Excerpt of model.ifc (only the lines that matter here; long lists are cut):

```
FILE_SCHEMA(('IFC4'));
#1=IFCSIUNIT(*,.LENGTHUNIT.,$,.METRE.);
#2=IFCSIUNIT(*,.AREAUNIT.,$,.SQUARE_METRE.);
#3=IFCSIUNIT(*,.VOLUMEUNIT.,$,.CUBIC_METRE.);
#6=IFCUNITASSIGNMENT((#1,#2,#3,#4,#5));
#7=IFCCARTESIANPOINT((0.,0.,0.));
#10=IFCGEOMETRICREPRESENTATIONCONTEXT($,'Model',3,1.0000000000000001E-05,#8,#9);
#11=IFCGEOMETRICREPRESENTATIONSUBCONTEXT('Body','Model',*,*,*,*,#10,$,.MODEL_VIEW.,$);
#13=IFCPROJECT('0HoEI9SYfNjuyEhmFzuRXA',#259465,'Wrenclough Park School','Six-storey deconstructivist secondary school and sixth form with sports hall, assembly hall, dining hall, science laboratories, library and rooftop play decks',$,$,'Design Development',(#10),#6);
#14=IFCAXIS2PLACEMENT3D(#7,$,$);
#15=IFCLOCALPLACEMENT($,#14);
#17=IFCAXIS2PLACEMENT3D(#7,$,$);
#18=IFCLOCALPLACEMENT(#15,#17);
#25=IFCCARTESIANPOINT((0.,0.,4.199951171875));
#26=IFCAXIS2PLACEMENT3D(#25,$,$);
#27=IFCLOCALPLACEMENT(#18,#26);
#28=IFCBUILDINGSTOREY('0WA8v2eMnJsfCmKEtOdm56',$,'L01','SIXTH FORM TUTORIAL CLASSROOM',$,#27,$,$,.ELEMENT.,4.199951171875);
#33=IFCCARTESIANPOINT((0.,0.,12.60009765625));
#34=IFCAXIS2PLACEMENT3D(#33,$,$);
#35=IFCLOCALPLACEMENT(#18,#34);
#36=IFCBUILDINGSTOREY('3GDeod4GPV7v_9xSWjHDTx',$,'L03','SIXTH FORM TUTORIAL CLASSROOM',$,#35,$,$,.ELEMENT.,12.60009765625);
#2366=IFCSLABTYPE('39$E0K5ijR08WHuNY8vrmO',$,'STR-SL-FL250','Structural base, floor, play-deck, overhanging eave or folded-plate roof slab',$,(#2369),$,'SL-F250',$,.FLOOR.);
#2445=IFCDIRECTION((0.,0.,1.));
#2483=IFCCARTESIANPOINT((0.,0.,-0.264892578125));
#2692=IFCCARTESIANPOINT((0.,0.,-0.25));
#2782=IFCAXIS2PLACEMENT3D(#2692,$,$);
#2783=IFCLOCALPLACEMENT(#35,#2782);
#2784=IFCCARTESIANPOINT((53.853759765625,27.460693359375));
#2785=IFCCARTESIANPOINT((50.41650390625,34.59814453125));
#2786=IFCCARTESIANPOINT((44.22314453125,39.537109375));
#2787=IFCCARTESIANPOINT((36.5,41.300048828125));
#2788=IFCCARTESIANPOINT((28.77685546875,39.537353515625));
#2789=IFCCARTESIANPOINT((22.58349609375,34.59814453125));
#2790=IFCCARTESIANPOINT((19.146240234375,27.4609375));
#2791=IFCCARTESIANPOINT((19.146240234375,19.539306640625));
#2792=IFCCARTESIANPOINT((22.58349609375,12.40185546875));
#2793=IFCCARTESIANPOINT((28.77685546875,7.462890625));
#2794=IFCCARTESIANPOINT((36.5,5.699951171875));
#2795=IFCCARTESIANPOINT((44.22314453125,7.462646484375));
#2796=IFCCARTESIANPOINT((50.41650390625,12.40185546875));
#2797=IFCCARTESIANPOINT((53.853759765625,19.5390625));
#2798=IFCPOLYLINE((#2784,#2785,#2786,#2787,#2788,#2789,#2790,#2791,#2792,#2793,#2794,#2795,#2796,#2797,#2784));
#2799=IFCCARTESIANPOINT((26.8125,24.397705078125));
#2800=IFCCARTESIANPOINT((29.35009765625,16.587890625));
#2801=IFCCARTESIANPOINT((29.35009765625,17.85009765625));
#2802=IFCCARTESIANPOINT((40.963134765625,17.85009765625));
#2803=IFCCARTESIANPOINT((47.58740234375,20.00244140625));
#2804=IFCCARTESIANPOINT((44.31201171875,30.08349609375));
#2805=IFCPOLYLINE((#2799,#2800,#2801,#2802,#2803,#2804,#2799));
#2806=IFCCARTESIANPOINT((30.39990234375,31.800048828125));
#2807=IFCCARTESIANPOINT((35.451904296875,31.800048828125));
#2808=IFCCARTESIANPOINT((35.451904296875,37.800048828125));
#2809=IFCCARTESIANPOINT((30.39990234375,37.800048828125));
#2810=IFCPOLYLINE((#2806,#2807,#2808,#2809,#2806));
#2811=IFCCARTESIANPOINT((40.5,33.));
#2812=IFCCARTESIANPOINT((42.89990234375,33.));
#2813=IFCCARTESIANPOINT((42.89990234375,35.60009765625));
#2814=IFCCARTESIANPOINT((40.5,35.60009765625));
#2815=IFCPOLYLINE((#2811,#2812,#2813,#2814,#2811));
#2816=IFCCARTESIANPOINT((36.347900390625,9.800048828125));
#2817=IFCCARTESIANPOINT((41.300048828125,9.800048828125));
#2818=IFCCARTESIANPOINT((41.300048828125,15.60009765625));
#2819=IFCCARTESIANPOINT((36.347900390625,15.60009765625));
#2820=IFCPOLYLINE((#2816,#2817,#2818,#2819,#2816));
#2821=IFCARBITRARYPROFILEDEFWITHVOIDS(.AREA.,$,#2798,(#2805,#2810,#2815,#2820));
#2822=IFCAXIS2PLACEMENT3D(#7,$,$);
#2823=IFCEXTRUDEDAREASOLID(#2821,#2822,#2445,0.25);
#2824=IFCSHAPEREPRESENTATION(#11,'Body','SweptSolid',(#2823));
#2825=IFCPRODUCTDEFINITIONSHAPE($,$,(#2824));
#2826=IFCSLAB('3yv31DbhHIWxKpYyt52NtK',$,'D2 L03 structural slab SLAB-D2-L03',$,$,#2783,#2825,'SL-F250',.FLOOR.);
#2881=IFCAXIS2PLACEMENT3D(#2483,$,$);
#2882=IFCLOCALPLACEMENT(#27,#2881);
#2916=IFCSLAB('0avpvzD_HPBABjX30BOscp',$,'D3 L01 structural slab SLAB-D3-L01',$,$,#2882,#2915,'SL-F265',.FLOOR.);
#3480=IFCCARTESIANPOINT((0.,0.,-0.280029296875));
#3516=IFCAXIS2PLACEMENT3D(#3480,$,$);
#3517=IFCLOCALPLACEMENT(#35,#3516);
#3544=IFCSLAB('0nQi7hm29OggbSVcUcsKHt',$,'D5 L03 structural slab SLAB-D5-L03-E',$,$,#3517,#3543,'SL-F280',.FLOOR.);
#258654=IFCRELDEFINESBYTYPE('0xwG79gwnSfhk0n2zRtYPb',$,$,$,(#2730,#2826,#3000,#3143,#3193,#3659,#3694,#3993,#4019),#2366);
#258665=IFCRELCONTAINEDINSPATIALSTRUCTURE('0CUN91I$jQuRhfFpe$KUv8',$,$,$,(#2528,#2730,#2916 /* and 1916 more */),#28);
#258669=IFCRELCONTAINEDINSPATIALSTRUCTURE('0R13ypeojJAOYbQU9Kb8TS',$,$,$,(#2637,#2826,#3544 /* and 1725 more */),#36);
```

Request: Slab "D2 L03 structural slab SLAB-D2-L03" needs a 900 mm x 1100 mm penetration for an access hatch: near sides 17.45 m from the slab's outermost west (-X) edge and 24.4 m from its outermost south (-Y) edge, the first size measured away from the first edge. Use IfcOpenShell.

```python
import numpy as np
import ifcopenshell
import ifcopenshell.api.feature
import ifcopenshell.api.geometry
import ifcopenshell.api.root
import ifcopenshell.geom
import ifcopenshell.util.placement
import ifcopenshell.util.representation
import ifcopenshell.util.shape
import ifcopenshell.util.unit

model = ifcopenshell.open("model.ifc")
unit_scale = ifcopenshell.util.unit.calculate_unit_scale(model)
settings = ifcopenshell.geom.settings()


def volume(element):
    """Net volume in cubic metres, openings subtracted."""
    shape = ifcopenshell.geom.create_shape(settings, element)
    return ifcopenshell.util.shape.get_volume(shape.geometry)


slab = model.by_guid("3yv31DbhHIWxKpYyt52NtK")
before = volume(slab)

# Extent in the slab's own axes, in metres. The edges named are its -X and -Y sides.
slab_shape = ifcopenshell.geom.create_shape(settings, slab)
vertices = ifcopenshell.util.shape.get_vertices(slab_shape.geometry)
x_min, y_min, bottom = vertices.min(axis=0)
top = vertices[:, 2].max()

opening = ifcopenshell.api.root.create_entity(model, ifc_class="IfcOpeningElement", name="Access hatch opening", predefined_type="OPENING")
context = ifcopenshell.util.representation.get_context(model, "Model", "Body", "MODEL_VIEW")
width, depth = 0.9, 1.1
outline = [(0.0, 0.0), (width, 0.0), (width, depth), (0.0, depth), (0.0, 0.0)]
# Overshoot both faces by 50 mm so the cut is clean.
shape = ifcopenshell.api.geometry.add_slab_representation(
    model, context=context, depth=top - bottom + 0.1, polyline=outline
)
ifcopenshell.api.geometry.assign_representation(model, product=opening, representation=shape)

matrix = ifcopenshell.util.placement.get_local_placement(slab.ObjectPlacement)
matrix[:, 3] = matrix @ np.append(np.array([x_min + 17.45, y_min + 24.4, bottom - 0.05]) / unit_scale, 1.0)
ifcopenshell.api.geometry.edit_object_placement(model, product=opening, matrix=matrix, is_si=False)
ifcopenshell.api.feature.add_feature(model, feature=opening, element=slab)

after = volume(slab)

print(f"slab volume {before:.3f} -> {after:.3f} m3")

model.write("model_updated.ifc")
```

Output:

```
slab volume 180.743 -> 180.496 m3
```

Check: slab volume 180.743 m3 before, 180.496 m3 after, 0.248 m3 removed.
